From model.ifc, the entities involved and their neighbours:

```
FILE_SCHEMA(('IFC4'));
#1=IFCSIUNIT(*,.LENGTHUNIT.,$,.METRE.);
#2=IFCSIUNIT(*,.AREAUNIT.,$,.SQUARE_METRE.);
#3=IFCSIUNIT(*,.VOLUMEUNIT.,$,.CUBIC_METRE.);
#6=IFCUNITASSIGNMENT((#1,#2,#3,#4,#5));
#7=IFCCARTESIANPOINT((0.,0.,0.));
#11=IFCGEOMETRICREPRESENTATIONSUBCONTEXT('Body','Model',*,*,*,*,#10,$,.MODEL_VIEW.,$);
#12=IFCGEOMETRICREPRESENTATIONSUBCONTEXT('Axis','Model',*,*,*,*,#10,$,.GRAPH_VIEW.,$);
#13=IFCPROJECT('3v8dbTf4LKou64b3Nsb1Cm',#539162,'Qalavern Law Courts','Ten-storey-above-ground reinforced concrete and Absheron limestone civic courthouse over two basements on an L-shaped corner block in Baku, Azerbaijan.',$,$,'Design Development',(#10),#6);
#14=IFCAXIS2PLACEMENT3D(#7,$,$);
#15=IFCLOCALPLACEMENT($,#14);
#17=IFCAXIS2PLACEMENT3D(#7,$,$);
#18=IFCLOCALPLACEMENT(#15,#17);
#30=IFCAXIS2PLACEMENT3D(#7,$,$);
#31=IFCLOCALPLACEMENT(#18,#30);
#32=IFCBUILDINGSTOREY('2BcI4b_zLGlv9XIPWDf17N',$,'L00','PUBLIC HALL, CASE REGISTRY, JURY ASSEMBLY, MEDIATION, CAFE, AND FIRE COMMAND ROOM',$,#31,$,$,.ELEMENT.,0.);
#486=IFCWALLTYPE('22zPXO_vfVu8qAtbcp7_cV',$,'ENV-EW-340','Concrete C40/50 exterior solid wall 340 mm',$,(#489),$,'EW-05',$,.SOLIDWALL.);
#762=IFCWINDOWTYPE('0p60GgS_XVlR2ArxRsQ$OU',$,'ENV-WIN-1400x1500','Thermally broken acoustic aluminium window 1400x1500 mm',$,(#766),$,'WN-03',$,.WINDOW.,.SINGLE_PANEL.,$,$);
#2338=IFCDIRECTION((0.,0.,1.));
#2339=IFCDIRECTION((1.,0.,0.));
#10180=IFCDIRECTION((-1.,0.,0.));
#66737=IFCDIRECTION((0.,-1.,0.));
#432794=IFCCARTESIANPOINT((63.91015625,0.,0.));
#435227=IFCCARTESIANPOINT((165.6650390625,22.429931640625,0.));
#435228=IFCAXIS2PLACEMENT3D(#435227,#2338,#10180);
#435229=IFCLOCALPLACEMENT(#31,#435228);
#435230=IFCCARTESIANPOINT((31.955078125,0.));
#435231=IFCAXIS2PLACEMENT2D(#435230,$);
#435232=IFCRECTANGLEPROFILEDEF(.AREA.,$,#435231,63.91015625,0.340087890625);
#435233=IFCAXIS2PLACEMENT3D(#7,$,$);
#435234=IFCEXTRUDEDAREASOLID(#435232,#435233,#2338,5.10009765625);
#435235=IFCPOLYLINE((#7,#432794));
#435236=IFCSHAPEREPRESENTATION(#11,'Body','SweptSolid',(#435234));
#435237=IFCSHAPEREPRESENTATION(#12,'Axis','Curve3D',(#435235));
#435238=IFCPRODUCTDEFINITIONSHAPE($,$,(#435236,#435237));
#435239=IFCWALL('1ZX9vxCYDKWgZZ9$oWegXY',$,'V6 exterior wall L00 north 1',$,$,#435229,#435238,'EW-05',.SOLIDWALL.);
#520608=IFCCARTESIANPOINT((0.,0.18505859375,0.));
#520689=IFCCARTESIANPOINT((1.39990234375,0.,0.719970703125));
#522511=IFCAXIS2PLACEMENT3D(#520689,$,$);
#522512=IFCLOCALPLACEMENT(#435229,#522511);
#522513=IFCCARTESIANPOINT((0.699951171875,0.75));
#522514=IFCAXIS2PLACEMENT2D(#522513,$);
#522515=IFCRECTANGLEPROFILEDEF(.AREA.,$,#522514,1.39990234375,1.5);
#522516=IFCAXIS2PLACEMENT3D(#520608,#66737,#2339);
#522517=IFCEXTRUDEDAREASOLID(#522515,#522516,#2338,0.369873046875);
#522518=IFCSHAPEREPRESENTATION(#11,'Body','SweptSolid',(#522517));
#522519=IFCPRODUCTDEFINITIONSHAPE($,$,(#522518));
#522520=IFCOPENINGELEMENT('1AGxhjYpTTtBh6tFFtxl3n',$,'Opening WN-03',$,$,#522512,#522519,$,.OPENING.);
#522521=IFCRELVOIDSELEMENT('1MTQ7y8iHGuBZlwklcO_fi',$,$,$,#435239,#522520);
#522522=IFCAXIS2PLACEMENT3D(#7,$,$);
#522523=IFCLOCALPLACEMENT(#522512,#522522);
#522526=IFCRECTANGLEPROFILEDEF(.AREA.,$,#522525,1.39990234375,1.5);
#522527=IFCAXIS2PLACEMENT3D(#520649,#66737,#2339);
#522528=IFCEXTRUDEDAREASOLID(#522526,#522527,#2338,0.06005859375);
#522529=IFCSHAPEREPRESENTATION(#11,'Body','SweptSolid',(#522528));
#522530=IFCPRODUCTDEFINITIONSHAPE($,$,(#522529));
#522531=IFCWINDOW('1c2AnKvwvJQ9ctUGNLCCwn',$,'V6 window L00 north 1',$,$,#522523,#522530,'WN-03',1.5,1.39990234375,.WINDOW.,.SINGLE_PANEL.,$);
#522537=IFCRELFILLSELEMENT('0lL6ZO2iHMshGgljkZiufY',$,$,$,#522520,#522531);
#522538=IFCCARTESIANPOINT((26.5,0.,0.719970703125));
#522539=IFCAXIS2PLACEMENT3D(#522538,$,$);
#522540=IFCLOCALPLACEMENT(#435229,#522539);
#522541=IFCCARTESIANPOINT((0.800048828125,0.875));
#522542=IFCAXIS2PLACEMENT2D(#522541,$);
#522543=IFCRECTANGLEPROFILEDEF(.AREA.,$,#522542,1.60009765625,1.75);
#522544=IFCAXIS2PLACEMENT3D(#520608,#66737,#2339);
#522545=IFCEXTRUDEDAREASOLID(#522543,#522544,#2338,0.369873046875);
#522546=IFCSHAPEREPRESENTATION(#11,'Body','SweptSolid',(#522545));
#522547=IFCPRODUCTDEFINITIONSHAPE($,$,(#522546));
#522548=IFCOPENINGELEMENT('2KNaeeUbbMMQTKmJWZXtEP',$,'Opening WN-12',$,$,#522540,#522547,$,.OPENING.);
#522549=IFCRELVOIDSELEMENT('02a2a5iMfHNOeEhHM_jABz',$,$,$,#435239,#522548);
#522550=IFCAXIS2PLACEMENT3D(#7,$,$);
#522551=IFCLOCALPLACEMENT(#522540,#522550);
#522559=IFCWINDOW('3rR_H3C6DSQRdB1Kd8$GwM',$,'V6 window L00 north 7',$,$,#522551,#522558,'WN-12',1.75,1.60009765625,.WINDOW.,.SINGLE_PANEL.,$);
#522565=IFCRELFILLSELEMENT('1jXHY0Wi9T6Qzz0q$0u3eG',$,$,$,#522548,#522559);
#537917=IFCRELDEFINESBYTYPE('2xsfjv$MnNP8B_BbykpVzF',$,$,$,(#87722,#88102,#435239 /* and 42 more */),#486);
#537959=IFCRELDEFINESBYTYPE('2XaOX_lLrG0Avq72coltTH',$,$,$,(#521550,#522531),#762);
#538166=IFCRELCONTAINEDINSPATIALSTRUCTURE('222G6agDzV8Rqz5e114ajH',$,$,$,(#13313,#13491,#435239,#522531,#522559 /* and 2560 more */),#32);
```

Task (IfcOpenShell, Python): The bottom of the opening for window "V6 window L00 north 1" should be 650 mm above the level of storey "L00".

```python
import numpy as np
import ifcopenshell
import ifcopenshell.api.geometry
import ifcopenshell.geom
import ifcopenshell.util.element
import ifcopenshell.util.placement
import ifcopenshell.util.shape
import ifcopenshell.util.unit

model = ifcopenshell.open("model.ifc")
unit_scale = ifcopenshell.util.unit.calculate_unit_scale(model)

window = model.by_guid("1c2AnKvwvJQ9ctUGNLCCwn")
opening = window.FillsVoids[0].RelatingOpeningElement
storey = ifcopenshell.util.element.get_container(window, ifc_class="IfcBuildingStorey")
level = ifcopenshell.util.placement.get_local_placement(storey.ObjectPlacement)[2, 3]

# The opening's origin need not be at the sill, so measure its lowest point.
shape = ifcopenshell.geom.create_shape(ifcopenshell.geom.settings(), opening)
bottom = ifcopenshell.util.shape.get_shape_bottom_elevation(shape, shape.geometry) / unit_scale
dz = level + 0.65 - bottom

shift = np.array([0.0, 0.0, dz])
# The window is placed relative to its opening, so it follows when the opening moves.
matrix = ifcopenshell.util.placement.get_local_placement(opening.ObjectPlacement)
matrix[:3, 3] += shift
ifcopenshell.api.geometry.edit_object_placement(
    model, product=opening, matrix=matrix, is_si=False, should_transform_children=True
)

print(f"moved by {dz * unit_scale:+.3f} m")

model.write("model-out.ifc")
```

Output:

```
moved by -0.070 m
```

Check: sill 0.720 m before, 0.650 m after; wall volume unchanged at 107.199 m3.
